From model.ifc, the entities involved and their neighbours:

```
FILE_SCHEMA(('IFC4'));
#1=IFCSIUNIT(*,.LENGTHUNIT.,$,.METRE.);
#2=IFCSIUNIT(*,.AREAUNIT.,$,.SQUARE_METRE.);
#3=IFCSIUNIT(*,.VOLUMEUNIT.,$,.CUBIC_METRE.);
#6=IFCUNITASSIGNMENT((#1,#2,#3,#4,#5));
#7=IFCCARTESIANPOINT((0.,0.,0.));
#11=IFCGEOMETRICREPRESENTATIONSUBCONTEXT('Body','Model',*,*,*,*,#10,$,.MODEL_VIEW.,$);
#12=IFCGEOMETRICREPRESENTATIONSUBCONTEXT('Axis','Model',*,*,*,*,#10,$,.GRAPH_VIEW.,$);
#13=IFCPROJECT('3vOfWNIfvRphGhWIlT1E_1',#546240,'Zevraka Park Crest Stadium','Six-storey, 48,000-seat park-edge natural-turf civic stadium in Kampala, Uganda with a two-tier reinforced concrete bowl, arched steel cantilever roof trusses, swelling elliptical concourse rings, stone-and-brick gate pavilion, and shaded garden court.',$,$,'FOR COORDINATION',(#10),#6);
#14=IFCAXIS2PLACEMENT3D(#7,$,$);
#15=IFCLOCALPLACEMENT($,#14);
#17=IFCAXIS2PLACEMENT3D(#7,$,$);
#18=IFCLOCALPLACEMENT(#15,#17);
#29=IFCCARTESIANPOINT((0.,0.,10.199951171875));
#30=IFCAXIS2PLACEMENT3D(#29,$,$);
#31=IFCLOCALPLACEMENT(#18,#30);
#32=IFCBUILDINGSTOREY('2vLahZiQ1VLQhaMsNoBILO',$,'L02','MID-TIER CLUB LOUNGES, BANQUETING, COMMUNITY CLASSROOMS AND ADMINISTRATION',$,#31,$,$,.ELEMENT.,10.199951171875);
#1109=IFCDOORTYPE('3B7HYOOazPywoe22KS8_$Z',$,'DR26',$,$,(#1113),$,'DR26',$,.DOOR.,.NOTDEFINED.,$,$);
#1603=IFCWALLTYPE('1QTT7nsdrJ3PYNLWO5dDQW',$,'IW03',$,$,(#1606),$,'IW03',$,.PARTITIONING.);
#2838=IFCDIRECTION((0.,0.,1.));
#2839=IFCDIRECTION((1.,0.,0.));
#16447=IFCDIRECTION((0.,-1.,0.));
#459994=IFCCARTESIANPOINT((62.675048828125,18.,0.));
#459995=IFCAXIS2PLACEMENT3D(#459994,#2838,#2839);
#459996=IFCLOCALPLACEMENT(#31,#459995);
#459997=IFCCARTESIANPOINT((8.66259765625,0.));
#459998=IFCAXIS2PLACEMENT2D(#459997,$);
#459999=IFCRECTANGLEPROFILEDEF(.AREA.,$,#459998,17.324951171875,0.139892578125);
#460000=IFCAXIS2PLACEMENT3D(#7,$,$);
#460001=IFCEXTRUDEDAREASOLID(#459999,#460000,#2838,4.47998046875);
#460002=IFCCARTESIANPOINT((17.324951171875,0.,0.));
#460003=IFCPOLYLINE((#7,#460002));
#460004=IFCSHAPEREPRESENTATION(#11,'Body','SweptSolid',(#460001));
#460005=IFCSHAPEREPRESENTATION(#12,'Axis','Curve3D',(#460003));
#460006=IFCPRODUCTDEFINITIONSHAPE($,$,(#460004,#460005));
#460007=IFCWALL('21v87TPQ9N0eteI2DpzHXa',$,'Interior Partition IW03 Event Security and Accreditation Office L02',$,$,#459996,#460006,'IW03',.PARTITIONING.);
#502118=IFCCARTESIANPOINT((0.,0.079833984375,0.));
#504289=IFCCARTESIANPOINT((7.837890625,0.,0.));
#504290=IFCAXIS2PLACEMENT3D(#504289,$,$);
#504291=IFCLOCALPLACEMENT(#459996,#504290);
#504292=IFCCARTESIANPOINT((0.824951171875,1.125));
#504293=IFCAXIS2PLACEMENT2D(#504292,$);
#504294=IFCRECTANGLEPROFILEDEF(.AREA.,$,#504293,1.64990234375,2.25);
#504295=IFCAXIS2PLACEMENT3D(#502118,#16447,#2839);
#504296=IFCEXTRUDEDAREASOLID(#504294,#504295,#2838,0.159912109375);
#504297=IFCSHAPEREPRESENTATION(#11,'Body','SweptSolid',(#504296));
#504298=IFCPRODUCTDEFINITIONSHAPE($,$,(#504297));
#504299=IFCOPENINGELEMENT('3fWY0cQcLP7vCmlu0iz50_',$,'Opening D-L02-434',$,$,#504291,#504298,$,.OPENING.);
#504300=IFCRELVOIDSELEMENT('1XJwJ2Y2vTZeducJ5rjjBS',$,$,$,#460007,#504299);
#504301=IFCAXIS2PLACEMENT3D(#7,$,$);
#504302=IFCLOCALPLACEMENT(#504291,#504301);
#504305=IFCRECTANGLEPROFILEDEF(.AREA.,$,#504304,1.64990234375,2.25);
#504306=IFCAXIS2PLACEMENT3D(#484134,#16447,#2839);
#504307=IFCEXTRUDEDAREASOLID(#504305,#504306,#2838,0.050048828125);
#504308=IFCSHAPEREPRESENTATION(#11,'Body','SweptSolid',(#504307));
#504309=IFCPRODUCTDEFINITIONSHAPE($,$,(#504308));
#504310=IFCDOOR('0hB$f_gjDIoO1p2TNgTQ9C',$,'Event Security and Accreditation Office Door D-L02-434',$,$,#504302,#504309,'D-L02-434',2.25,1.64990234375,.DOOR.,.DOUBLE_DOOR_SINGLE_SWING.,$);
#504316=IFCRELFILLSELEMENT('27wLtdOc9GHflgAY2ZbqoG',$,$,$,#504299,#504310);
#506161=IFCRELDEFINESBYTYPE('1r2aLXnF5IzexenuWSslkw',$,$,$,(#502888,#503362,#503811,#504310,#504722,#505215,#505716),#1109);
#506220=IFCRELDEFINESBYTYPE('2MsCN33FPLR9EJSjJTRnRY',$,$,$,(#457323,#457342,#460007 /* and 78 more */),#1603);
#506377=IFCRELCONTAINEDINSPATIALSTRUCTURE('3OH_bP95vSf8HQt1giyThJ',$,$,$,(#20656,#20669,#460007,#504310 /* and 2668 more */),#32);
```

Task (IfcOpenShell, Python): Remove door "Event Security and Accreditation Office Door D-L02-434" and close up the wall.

```python
import ifcopenshell
import ifcopenshell.api.feature
import ifcopenshell.api.root
import ifcopenshell.geom
import ifcopenshell.util.shape

model = ifcopenshell.open("model.ifc")
settings = ifcopenshell.geom.settings()


def volume(element):
    """Net volume in cubic metres, openings subtracted."""
    shape = ifcopenshell.geom.create_shape(settings, element)
    return ifcopenshell.util.shape.get_volume(shape.geometry)


door = model.by_guid("0hB$f_gjDIoO1p2TNgTQ9C")
opening = door.FillsVoids[0].RelatingOpeningElement
wall = opening.VoidsElements[0].RelatingBuildingElement
before = volume(wall)

ifcopenshell.api.root.remove_product(model, product=door)
ifcopenshell.api.feature.remove_feature(model, feature=opening)

after = volume(wall)

print(f"wall volume {before:.3f} -> {after:.3f} m3")

model.write("model-out.ifc")
```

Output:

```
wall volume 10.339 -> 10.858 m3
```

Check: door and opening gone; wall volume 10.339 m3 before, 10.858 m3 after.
